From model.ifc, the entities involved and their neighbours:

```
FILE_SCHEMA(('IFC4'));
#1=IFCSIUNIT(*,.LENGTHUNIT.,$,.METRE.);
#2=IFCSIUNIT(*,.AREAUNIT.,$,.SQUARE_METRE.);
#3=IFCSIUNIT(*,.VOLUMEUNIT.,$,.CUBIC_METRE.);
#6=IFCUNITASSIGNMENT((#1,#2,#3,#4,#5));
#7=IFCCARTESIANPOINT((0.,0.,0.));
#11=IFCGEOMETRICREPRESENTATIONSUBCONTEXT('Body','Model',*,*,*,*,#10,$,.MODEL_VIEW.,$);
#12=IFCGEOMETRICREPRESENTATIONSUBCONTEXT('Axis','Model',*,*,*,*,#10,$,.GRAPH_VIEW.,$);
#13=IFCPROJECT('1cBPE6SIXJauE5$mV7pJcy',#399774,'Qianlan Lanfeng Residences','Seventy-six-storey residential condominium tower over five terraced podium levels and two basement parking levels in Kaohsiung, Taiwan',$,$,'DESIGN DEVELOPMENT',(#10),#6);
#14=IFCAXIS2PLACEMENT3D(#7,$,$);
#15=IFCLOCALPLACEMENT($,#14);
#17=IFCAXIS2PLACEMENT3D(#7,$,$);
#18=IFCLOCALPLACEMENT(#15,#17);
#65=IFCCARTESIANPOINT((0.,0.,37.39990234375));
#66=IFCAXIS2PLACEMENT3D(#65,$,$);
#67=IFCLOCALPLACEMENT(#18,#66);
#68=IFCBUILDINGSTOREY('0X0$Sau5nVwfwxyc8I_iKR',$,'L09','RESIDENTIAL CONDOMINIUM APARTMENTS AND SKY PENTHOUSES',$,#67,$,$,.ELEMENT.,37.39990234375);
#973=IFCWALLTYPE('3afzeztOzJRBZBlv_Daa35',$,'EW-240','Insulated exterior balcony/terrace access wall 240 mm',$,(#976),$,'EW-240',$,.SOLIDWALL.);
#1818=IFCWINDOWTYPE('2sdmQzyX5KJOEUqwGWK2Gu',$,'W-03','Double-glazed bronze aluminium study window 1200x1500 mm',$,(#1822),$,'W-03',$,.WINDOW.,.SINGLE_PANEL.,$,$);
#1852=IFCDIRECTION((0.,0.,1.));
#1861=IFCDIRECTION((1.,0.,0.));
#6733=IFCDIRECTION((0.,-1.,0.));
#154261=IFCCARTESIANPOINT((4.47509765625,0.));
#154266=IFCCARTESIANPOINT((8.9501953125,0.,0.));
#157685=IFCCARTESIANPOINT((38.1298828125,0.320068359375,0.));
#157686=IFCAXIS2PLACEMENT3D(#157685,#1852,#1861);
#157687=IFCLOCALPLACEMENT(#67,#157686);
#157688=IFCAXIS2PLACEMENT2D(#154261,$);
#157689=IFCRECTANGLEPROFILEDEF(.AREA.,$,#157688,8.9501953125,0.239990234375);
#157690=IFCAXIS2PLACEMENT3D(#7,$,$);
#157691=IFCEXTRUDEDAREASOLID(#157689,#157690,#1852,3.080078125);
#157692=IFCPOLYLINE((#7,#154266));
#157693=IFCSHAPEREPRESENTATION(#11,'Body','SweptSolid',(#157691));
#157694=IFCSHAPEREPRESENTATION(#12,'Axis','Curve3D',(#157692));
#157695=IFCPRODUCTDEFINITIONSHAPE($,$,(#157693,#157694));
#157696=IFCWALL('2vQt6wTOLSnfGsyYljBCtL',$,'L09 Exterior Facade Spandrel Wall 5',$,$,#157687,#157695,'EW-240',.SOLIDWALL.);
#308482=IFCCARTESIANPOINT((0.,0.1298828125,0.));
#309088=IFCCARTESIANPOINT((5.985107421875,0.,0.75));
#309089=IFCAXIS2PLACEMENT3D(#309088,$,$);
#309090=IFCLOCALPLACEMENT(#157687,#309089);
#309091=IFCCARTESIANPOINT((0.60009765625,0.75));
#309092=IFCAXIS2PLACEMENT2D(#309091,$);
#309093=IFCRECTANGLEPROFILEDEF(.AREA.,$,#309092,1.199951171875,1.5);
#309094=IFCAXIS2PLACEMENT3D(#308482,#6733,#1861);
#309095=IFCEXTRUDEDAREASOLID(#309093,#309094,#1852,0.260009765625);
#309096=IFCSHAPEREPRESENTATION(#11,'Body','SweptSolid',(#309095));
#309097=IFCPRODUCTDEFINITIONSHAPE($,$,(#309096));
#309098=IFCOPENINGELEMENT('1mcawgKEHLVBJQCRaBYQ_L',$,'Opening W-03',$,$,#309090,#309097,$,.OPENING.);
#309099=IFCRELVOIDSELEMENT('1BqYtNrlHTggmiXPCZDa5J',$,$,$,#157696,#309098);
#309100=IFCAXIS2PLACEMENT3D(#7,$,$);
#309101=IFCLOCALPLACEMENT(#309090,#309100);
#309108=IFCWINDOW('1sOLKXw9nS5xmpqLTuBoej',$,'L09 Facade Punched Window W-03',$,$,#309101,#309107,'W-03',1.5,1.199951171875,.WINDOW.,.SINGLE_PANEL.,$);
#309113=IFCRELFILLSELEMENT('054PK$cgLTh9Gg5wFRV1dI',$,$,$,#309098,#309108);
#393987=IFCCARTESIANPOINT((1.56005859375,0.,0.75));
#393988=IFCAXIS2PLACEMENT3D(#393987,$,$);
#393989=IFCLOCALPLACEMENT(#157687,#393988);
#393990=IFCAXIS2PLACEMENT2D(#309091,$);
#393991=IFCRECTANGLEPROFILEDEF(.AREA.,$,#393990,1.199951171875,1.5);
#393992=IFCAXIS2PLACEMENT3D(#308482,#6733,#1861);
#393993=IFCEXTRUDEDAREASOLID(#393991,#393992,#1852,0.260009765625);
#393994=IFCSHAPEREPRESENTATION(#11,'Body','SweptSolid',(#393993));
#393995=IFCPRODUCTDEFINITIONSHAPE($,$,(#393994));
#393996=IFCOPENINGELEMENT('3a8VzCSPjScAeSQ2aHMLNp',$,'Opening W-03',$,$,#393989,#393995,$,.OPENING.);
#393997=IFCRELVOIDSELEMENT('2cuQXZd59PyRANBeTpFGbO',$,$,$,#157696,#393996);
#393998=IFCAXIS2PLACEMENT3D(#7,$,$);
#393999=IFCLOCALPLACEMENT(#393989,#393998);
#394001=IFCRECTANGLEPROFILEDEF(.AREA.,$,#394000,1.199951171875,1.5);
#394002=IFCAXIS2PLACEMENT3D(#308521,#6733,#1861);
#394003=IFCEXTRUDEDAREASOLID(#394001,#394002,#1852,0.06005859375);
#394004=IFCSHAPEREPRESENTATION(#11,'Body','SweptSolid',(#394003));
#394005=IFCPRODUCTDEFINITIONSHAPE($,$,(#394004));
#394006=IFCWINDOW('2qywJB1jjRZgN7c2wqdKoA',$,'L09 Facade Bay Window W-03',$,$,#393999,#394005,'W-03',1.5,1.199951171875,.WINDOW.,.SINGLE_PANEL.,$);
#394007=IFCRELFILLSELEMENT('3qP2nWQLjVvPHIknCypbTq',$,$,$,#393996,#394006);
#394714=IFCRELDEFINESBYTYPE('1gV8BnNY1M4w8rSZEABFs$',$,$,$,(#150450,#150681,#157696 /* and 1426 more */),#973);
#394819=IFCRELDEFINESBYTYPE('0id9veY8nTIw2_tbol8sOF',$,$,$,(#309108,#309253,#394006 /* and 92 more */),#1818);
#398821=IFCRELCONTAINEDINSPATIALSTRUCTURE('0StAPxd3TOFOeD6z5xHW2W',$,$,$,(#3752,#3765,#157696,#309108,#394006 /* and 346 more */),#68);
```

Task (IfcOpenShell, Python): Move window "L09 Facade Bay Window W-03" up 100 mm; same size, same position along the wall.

```python
import numpy as np
import ifcopenshell
import ifcopenshell.api.geometry
import ifcopenshell.util.placement
import ifcopenshell.util.unit

model = ifcopenshell.open("model.ifc")
unit_scale = ifcopenshell.util.unit.calculate_unit_scale(model)

window = model.by_id(394006)
opening = window.FillsVoids[0].RelatingOpeningElement
dz = 0.1 / unit_scale

shift = np.array([0.0, 0.0, dz])
# The window is placed relative to its opening, so it follows when the opening moves.
matrix = ifcopenshell.util.placement.get_local_placement(opening.ObjectPlacement)
matrix[:3, 3] += shift
ifcopenshell.api.geometry.edit_object_placement(
    model, product=opening, matrix=matrix, is_si=False, should_transform_children=True
)

print(f"moved by {dz * unit_scale:+.3f} m")

model.write("model_updated.ifc")
```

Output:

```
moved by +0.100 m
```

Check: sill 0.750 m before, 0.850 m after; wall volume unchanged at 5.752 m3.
